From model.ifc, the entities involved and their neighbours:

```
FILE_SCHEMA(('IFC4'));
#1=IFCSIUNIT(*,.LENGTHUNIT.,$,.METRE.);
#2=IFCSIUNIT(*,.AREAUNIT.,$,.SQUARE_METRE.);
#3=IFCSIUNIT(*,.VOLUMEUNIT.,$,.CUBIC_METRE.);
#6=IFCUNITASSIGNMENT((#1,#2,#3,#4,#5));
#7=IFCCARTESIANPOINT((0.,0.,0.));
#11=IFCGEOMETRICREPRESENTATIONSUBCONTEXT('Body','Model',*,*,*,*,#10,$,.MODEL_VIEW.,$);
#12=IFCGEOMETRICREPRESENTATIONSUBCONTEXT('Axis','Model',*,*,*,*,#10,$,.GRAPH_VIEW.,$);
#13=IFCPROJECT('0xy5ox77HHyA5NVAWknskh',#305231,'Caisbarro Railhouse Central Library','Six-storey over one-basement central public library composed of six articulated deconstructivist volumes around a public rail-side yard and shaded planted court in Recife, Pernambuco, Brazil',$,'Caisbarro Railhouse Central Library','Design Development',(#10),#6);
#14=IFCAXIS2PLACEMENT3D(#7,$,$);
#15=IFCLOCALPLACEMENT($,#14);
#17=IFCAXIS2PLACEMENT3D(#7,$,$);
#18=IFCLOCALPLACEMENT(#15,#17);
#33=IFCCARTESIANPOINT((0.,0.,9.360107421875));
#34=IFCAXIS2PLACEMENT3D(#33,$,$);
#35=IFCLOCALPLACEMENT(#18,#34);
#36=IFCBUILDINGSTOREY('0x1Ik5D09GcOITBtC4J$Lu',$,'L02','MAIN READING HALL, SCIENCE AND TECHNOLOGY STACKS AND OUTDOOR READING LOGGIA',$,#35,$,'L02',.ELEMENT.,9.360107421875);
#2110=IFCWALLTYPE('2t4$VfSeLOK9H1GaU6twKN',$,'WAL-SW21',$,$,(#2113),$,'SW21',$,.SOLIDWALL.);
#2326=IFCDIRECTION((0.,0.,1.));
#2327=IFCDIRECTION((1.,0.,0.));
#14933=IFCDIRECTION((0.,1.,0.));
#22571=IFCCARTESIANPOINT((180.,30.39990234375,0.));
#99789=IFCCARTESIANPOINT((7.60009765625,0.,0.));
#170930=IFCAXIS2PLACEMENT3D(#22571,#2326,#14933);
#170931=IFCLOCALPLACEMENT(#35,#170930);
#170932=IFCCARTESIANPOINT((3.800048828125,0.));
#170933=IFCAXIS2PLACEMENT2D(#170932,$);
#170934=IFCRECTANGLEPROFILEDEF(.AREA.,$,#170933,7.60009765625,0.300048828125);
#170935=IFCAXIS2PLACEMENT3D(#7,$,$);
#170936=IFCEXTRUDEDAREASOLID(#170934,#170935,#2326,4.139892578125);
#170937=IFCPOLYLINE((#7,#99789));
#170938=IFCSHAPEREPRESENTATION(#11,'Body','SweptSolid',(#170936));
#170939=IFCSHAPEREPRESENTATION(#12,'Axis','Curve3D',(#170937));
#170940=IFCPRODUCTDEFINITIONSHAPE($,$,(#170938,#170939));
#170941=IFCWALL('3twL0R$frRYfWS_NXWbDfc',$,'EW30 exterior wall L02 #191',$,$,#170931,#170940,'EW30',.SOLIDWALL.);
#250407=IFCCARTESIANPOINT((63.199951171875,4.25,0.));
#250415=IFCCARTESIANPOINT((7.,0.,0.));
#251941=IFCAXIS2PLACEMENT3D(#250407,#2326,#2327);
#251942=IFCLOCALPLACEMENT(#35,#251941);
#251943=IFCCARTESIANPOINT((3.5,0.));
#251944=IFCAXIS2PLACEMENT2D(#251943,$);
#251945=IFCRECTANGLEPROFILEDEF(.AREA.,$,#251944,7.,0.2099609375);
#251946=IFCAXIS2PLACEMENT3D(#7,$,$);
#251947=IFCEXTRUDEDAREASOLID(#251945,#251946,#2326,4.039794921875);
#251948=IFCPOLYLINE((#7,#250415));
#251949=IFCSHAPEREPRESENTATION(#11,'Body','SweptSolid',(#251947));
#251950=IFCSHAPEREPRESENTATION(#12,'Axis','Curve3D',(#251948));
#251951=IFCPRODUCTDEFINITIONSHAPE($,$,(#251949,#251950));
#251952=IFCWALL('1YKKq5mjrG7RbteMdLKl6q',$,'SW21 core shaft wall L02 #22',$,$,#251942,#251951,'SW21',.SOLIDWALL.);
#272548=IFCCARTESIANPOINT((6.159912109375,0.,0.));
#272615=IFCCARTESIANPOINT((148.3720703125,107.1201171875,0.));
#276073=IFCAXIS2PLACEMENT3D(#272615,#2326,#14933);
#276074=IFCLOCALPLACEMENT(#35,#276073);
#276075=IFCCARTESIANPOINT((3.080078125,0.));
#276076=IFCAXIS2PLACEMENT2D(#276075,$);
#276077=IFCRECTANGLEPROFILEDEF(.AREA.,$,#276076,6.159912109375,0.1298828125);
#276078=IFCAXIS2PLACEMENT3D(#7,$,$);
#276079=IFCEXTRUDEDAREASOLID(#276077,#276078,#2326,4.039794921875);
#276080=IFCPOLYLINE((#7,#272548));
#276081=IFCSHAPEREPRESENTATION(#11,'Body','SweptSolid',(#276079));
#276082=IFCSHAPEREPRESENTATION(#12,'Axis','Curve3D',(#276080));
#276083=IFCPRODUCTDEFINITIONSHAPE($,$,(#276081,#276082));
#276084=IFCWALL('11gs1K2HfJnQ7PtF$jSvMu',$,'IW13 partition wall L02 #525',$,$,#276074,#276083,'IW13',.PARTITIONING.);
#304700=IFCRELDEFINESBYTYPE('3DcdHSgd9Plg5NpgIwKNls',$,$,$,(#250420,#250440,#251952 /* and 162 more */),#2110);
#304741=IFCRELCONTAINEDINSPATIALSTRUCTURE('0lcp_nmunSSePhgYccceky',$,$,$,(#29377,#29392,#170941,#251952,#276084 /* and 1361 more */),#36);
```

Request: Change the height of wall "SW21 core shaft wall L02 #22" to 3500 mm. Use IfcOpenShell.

```python
import ifcopenshell
import ifcopenshell.geom
import ifcopenshell.util.representation
import ifcopenshell.util.shape
import ifcopenshell.util.unit

model = ifcopenshell.open("model.ifc")
unit_scale = ifcopenshell.util.unit.calculate_unit_scale(model)
settings = ifcopenshell.geom.settings()


def volume(element):
    """Net volume in cubic metres, openings subtracted."""
    shape = ifcopenshell.geom.create_shape(settings, element)
    return ifcopenshell.util.shape.get_volume(shape.geometry)


wall = model.by_guid("1YKKq5mjrG7RbteMdLKl6q")
before = volume(wall)

body = ifcopenshell.util.representation.get_representation(wall, "Model", "Body")
solid = body.Items[0]
old_height = solid.Depth
solid.Depth = 3.5 / unit_scale
after = volume(wall)

print(f"height {old_height:g} -> {solid.Depth:g}, volume {before:.3f} -> {after:.3f} m3")

model.write("model_edited.ifc")
```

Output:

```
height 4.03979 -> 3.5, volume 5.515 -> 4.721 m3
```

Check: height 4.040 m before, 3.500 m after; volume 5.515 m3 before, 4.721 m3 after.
